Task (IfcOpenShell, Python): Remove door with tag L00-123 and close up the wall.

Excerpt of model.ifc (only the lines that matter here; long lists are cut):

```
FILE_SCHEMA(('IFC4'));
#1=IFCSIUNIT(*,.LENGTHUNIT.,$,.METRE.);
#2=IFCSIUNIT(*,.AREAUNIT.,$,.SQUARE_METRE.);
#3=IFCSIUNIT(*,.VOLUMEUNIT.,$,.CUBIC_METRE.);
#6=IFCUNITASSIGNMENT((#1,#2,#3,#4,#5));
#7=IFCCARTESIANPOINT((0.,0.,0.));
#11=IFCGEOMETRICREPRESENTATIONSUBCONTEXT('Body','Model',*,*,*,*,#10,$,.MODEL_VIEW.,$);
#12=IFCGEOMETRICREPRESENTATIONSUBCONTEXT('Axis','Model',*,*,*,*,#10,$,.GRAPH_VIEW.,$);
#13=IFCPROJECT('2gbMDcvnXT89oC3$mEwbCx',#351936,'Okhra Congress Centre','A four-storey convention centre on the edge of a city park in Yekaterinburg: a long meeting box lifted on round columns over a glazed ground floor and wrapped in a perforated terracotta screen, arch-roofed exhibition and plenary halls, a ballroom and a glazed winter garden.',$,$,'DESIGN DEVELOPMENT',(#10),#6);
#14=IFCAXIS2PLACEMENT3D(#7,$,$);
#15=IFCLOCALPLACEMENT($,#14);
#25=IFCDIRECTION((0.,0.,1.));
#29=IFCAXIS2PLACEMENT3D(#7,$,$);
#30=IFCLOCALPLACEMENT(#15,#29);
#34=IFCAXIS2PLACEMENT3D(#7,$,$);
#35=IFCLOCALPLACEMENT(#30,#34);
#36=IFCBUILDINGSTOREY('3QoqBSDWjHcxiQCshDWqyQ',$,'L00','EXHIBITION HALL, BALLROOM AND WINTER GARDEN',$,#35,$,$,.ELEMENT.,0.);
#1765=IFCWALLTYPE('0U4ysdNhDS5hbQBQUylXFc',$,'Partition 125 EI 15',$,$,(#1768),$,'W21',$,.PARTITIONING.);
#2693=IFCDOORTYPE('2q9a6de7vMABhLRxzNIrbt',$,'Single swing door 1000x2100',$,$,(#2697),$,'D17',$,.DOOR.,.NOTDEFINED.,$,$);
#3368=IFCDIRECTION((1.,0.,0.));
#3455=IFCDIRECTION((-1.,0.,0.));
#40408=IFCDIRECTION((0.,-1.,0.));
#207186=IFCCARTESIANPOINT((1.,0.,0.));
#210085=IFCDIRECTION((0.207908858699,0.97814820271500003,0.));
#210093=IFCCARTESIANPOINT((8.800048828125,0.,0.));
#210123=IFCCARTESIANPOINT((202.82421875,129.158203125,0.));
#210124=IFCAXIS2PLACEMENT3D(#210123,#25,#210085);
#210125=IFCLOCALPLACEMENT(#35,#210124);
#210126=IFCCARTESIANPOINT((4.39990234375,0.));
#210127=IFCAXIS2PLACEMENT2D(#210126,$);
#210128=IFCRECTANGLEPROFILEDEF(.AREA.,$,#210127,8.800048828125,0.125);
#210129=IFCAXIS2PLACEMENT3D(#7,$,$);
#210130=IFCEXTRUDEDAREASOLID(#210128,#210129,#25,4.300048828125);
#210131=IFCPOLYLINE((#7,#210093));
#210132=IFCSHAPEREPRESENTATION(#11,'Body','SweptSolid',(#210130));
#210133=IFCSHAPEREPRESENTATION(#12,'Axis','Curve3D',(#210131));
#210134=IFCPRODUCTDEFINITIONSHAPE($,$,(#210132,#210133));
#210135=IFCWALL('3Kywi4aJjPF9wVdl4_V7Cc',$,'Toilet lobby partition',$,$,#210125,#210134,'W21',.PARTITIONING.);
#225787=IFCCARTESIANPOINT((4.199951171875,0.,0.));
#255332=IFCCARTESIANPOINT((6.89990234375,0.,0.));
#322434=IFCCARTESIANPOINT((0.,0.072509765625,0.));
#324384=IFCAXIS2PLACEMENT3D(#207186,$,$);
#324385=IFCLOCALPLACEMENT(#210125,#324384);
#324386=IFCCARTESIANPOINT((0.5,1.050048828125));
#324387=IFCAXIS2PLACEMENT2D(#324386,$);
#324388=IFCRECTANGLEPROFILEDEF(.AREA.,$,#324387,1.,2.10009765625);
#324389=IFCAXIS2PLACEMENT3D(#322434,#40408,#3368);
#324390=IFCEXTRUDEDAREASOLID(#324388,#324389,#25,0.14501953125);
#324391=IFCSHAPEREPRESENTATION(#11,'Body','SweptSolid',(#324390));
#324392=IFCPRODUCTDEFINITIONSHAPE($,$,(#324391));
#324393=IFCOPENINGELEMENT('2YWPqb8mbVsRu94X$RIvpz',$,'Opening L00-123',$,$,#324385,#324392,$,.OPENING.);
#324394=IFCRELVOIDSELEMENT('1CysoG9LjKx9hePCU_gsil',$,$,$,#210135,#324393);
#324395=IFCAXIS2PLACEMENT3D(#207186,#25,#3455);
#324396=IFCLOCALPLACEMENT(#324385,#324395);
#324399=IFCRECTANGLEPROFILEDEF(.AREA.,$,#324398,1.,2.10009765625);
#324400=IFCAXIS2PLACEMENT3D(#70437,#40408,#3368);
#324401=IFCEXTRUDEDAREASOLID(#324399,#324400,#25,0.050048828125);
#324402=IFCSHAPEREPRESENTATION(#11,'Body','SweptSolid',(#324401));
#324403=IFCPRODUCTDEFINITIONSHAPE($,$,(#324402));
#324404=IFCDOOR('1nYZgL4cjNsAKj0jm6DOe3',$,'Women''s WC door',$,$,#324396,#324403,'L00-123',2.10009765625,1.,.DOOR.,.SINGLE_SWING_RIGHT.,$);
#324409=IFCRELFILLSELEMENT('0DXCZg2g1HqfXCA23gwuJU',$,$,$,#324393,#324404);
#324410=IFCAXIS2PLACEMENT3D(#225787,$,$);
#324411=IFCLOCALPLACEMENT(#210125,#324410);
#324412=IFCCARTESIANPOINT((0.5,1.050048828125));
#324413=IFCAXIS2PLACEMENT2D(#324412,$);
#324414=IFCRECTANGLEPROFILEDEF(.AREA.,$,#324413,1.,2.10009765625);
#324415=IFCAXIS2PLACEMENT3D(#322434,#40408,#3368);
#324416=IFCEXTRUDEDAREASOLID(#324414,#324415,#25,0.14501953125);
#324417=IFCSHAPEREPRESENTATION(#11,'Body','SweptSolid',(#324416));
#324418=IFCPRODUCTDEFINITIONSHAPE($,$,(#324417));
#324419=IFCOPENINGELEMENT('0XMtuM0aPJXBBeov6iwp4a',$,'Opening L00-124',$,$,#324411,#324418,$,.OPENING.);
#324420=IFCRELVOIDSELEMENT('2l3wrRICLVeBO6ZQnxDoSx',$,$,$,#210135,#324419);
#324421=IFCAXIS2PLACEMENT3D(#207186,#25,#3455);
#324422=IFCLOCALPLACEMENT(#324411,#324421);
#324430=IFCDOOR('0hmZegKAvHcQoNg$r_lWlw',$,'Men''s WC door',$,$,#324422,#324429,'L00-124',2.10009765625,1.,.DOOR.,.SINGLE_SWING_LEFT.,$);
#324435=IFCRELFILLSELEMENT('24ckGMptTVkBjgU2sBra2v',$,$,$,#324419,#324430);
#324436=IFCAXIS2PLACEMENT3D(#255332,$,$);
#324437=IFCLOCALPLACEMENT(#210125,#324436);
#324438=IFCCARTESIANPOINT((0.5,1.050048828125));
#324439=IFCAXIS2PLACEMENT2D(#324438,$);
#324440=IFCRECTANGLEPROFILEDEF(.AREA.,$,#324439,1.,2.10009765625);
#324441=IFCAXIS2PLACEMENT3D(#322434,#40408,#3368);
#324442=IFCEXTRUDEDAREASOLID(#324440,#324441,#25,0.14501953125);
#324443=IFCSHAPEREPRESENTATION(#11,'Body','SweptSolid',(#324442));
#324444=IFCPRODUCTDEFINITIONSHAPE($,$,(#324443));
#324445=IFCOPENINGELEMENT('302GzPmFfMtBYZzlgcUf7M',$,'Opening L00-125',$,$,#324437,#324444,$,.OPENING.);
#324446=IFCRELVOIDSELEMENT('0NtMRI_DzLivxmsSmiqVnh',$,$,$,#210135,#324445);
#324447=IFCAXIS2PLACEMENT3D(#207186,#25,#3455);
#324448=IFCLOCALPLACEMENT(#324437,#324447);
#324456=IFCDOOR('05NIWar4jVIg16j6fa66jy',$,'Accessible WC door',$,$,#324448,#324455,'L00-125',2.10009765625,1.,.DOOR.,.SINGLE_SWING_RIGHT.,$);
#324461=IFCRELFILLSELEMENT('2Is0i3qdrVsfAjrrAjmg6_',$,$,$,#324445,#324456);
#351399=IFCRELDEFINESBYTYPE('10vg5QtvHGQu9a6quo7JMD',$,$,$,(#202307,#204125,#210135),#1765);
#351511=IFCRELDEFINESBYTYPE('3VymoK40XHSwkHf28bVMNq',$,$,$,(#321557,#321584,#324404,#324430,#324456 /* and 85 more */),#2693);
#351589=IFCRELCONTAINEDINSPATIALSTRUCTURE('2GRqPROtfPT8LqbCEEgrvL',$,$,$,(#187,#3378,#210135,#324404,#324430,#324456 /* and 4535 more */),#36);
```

```python
import ifcopenshell
import ifcopenshell.api.feature
import ifcopenshell.api.root
import ifcopenshell.geom
import ifcopenshell.util.shape

model = ifcopenshell.open("model.ifc")
settings = ifcopenshell.geom.settings()


def volume(element):
    """Net volume in cubic metres, openings subtracted."""
    shape = ifcopenshell.geom.create_shape(settings, element)
    return ifcopenshell.util.shape.get_volume(shape.geometry)


door = model.by_guid("1nYZgL4cjNsAKj0jm6DOe3")
opening = door.FillsVoids[0].RelatingOpeningElement
wall = opening.VoidsElements[0].RelatingBuildingElement
before = volume(wall)

ifcopenshell.api.root.remove_product(model, product=door)
ifcopenshell.api.feature.remove_feature(model, feature=opening)

after = volume(wall)

print(f"wall volume {before:.3f} -> {after:.3f} m3")

model.write("model_v2.ifc")
```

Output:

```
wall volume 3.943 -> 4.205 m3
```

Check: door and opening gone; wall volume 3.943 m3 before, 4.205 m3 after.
